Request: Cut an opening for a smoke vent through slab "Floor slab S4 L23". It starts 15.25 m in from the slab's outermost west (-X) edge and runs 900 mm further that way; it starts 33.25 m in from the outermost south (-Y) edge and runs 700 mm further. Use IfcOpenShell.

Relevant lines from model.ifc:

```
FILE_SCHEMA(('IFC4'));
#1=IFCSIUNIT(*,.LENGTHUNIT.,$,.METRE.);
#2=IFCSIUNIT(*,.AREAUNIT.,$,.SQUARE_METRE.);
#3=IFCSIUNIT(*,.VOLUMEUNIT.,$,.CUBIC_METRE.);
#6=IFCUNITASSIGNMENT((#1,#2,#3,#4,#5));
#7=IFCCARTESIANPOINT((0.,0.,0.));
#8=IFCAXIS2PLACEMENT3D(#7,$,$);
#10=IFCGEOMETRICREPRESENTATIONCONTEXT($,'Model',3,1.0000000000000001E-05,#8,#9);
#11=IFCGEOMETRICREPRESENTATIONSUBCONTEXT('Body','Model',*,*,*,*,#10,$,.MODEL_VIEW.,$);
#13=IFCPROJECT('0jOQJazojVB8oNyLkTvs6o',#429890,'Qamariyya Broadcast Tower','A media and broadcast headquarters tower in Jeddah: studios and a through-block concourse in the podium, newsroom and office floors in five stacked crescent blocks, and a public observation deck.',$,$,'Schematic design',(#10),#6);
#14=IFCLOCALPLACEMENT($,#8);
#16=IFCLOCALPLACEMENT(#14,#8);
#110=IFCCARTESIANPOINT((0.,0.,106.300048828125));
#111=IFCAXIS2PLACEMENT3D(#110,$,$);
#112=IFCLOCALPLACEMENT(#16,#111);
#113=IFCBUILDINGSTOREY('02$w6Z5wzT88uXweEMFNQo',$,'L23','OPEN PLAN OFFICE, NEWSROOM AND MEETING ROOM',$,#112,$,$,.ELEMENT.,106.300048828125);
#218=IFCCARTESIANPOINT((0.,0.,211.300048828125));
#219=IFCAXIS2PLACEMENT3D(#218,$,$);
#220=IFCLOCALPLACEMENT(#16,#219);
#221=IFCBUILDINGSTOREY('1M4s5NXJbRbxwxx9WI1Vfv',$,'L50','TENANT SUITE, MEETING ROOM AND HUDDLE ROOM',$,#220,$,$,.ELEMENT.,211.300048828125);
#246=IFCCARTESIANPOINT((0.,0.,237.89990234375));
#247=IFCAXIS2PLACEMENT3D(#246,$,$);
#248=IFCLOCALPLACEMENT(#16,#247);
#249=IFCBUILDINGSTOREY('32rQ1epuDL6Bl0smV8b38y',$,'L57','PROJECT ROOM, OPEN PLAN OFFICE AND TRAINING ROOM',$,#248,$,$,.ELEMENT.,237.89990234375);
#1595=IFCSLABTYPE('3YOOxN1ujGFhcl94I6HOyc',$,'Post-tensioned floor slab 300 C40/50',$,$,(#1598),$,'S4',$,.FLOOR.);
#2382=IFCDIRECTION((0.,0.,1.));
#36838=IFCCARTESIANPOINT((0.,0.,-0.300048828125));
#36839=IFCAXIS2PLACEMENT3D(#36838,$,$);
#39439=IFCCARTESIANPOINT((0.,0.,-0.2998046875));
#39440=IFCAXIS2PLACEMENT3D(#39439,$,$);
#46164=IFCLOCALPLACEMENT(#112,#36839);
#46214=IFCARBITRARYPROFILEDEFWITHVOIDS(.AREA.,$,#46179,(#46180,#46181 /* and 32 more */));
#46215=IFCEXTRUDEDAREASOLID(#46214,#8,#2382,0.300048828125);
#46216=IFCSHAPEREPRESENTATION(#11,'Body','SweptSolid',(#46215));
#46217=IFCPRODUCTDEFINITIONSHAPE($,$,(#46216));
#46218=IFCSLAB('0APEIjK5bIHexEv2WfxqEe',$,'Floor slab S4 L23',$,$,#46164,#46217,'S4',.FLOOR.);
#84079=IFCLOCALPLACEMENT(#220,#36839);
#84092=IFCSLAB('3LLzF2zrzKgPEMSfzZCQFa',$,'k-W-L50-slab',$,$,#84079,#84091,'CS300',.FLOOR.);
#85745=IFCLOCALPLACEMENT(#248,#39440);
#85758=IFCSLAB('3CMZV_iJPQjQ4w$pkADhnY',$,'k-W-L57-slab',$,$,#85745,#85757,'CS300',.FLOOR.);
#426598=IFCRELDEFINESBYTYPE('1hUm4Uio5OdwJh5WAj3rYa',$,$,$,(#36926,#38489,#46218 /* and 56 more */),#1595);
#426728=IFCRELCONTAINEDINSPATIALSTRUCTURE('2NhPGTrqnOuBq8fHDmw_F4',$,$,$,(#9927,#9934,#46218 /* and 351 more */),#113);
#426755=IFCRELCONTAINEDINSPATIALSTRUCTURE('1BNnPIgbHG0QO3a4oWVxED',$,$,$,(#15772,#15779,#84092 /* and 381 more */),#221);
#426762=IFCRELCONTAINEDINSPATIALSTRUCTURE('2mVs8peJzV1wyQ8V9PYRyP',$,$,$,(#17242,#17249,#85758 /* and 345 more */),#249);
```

```python
import numpy as np
import ifcopenshell
import ifcopenshell.api.feature
import ifcopenshell.api.geometry
import ifcopenshell.api.root
import ifcopenshell.geom
import ifcopenshell.util.placement
import ifcopenshell.util.representation
import ifcopenshell.util.shape
import ifcopenshell.util.unit

model = ifcopenshell.open("model.ifc")
unit_scale = ifcopenshell.util.unit.calculate_unit_scale(model)
settings = ifcopenshell.geom.settings()


def volume(element):
    """Net volume in cubic metres, openings subtracted."""
    shape = ifcopenshell.geom.create_shape(settings, element)
    return ifcopenshell.util.shape.get_volume(shape.geometry)


slab = model.by_guid("0APEIjK5bIHexEv2WfxqEe")
before = volume(slab)

# Extent in the slab's own axes, in metres. The edges named are its -X and -Y sides.
slab_shape = ifcopenshell.geom.create_shape(settings, slab)
vertices = ifcopenshell.util.shape.get_vertices(slab_shape.geometry)
x_min, y_min, bottom = vertices.min(axis=0)
top = vertices[:, 2].max()

opening = ifcopenshell.api.root.create_entity(model, ifc_class="IfcOpeningElement", name="Smoke vent opening", predefined_type="OPENING")
context = ifcopenshell.util.representation.get_context(model, "Model", "Body", "MODEL_VIEW")
width, depth = 0.9, 0.7
outline = [(0.0, 0.0), (width, 0.0), (width, depth), (0.0, depth), (0.0, 0.0)]
# Overshoot both faces by 50 mm so the cut is clean.
shape = ifcopenshell.api.geometry.add_slab_representation(
    model, context=context, depth=top - bottom + 0.1, polyline=outline
)
ifcopenshell.api.geometry.assign_representation(model, product=opening, representation=shape)

matrix = ifcopenshell.util.placement.get_local_placement(slab.ObjectPlacement)
matrix[:, 3] = matrix @ np.append(np.array([x_min + 15.25, y_min + 33.25, bottom - 0.05]) / unit_scale, 1.0)
ifcopenshell.api.geometry.edit_object_placement(model, product=opening, matrix=matrix, is_si=False)
ifcopenshell.api.feature.add_feature(model, feature=opening, element=slab)

after = volume(slab)

print(f"slab volume {before:.3f} -> {after:.3f} m3")

model.write("model_edited.ifc")
```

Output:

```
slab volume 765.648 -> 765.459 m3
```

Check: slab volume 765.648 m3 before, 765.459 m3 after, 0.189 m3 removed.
